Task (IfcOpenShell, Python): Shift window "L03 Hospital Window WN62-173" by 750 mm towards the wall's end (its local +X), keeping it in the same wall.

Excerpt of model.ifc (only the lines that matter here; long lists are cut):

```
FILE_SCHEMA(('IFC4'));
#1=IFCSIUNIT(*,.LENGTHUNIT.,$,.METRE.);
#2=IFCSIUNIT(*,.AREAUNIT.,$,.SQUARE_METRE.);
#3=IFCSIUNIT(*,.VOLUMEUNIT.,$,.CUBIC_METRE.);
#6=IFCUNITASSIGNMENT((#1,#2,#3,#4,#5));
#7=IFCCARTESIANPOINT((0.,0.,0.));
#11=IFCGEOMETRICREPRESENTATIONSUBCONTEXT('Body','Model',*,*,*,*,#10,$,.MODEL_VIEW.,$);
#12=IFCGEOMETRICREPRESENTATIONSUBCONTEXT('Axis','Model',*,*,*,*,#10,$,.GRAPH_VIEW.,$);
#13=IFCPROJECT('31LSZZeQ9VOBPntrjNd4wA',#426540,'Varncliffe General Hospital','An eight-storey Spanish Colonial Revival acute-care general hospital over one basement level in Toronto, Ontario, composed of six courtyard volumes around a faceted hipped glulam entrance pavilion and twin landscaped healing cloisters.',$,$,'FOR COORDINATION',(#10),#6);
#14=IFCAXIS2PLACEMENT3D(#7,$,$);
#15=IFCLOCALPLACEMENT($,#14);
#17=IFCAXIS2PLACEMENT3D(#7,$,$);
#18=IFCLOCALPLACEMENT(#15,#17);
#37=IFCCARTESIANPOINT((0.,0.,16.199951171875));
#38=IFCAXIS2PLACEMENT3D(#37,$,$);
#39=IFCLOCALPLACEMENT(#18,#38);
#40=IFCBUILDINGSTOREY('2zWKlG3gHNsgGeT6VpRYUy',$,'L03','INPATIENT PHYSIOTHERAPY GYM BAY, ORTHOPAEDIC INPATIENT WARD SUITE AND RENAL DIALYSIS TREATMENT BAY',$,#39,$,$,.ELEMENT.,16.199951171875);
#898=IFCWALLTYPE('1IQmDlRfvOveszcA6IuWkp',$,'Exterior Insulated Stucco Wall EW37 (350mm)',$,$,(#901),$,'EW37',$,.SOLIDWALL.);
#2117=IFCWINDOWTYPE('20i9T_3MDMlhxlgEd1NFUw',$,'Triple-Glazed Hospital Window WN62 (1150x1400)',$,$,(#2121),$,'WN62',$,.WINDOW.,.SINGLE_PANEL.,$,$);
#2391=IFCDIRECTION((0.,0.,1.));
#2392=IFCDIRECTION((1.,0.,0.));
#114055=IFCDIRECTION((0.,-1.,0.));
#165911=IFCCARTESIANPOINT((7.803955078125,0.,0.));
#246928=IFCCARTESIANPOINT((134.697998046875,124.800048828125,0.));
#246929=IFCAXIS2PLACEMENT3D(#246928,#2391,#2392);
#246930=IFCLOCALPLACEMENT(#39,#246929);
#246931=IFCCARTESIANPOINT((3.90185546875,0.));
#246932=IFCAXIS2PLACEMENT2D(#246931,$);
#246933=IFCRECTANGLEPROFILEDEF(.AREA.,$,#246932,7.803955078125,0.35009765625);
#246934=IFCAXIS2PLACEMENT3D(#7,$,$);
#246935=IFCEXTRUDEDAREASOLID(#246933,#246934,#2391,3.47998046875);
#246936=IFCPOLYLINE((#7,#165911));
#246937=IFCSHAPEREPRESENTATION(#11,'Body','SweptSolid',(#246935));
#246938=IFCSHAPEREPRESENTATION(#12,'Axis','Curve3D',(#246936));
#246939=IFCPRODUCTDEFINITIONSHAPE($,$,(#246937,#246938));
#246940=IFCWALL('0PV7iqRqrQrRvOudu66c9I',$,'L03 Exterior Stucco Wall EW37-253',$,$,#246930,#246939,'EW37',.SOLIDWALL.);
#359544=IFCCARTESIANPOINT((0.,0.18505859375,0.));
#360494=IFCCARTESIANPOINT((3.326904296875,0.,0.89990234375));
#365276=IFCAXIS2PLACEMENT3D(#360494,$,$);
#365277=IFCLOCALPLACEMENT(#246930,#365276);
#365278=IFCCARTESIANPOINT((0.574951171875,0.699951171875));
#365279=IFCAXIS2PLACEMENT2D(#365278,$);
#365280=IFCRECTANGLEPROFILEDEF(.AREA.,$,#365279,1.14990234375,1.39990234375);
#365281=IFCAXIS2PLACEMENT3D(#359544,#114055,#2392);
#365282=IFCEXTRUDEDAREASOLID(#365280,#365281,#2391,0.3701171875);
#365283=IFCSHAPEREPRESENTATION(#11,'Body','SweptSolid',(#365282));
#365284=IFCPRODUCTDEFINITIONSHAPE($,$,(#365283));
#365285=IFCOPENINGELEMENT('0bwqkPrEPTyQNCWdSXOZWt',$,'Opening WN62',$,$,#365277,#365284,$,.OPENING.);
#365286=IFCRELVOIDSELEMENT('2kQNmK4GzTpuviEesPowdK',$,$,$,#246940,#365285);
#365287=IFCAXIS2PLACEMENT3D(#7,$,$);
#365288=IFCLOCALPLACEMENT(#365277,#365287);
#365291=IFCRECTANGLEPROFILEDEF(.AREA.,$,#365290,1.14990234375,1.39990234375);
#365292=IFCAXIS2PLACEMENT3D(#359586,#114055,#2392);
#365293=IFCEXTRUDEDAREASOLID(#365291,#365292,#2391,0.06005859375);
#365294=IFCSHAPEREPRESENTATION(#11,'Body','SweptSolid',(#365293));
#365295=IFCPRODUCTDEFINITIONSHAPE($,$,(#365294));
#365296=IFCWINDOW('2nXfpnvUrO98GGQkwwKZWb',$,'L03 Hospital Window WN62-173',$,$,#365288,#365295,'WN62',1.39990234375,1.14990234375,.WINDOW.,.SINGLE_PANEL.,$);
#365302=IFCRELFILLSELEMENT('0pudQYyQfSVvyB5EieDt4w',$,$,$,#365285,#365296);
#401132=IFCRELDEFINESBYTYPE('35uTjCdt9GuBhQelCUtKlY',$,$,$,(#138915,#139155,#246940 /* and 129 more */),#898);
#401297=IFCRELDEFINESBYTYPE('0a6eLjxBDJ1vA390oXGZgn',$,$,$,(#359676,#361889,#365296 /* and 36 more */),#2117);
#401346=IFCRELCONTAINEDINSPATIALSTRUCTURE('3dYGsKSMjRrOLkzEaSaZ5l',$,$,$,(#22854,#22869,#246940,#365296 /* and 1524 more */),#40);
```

```python
import ifcopenshell
import ifcopenshell.api.geometry
import ifcopenshell.util.placement
import ifcopenshell.util.unit

model = ifcopenshell.open("model.ifc")
unit_scale = ifcopenshell.util.unit.calculate_unit_scale(model)

window = model.by_guid("2nXfpnvUrO98GGQkwwKZWb")
opening = window.FillsVoids[0].RelatingOpeningElement
wall = opening.VoidsElements[0].RelatingBuildingElement

wall_matrix = ifcopenshell.util.placement.get_local_placement(wall.ObjectPlacement)
shift = wall_matrix[:3, 0] * 0.75 / unit_scale
before = ifcopenshell.util.placement.get_local_placement(window.ObjectPlacement)[:3, 3].copy()

# The window is placed relative to its opening, so it follows when the opening moves.
matrix = ifcopenshell.util.placement.get_local_placement(opening.ObjectPlacement)
matrix[:3, 3] += shift
ifcopenshell.api.geometry.edit_object_placement(
    model, product=opening, matrix=matrix, is_si=False, should_transform_children=True
)

after = ifcopenshell.util.placement.get_local_placement(window.ObjectPlacement)[:3, 3]
print("window moved by", (after - before).round(3) + 0.0)

model.write("model_updated.ifc")
```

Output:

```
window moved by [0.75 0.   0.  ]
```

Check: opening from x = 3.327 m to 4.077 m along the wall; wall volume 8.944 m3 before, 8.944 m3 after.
